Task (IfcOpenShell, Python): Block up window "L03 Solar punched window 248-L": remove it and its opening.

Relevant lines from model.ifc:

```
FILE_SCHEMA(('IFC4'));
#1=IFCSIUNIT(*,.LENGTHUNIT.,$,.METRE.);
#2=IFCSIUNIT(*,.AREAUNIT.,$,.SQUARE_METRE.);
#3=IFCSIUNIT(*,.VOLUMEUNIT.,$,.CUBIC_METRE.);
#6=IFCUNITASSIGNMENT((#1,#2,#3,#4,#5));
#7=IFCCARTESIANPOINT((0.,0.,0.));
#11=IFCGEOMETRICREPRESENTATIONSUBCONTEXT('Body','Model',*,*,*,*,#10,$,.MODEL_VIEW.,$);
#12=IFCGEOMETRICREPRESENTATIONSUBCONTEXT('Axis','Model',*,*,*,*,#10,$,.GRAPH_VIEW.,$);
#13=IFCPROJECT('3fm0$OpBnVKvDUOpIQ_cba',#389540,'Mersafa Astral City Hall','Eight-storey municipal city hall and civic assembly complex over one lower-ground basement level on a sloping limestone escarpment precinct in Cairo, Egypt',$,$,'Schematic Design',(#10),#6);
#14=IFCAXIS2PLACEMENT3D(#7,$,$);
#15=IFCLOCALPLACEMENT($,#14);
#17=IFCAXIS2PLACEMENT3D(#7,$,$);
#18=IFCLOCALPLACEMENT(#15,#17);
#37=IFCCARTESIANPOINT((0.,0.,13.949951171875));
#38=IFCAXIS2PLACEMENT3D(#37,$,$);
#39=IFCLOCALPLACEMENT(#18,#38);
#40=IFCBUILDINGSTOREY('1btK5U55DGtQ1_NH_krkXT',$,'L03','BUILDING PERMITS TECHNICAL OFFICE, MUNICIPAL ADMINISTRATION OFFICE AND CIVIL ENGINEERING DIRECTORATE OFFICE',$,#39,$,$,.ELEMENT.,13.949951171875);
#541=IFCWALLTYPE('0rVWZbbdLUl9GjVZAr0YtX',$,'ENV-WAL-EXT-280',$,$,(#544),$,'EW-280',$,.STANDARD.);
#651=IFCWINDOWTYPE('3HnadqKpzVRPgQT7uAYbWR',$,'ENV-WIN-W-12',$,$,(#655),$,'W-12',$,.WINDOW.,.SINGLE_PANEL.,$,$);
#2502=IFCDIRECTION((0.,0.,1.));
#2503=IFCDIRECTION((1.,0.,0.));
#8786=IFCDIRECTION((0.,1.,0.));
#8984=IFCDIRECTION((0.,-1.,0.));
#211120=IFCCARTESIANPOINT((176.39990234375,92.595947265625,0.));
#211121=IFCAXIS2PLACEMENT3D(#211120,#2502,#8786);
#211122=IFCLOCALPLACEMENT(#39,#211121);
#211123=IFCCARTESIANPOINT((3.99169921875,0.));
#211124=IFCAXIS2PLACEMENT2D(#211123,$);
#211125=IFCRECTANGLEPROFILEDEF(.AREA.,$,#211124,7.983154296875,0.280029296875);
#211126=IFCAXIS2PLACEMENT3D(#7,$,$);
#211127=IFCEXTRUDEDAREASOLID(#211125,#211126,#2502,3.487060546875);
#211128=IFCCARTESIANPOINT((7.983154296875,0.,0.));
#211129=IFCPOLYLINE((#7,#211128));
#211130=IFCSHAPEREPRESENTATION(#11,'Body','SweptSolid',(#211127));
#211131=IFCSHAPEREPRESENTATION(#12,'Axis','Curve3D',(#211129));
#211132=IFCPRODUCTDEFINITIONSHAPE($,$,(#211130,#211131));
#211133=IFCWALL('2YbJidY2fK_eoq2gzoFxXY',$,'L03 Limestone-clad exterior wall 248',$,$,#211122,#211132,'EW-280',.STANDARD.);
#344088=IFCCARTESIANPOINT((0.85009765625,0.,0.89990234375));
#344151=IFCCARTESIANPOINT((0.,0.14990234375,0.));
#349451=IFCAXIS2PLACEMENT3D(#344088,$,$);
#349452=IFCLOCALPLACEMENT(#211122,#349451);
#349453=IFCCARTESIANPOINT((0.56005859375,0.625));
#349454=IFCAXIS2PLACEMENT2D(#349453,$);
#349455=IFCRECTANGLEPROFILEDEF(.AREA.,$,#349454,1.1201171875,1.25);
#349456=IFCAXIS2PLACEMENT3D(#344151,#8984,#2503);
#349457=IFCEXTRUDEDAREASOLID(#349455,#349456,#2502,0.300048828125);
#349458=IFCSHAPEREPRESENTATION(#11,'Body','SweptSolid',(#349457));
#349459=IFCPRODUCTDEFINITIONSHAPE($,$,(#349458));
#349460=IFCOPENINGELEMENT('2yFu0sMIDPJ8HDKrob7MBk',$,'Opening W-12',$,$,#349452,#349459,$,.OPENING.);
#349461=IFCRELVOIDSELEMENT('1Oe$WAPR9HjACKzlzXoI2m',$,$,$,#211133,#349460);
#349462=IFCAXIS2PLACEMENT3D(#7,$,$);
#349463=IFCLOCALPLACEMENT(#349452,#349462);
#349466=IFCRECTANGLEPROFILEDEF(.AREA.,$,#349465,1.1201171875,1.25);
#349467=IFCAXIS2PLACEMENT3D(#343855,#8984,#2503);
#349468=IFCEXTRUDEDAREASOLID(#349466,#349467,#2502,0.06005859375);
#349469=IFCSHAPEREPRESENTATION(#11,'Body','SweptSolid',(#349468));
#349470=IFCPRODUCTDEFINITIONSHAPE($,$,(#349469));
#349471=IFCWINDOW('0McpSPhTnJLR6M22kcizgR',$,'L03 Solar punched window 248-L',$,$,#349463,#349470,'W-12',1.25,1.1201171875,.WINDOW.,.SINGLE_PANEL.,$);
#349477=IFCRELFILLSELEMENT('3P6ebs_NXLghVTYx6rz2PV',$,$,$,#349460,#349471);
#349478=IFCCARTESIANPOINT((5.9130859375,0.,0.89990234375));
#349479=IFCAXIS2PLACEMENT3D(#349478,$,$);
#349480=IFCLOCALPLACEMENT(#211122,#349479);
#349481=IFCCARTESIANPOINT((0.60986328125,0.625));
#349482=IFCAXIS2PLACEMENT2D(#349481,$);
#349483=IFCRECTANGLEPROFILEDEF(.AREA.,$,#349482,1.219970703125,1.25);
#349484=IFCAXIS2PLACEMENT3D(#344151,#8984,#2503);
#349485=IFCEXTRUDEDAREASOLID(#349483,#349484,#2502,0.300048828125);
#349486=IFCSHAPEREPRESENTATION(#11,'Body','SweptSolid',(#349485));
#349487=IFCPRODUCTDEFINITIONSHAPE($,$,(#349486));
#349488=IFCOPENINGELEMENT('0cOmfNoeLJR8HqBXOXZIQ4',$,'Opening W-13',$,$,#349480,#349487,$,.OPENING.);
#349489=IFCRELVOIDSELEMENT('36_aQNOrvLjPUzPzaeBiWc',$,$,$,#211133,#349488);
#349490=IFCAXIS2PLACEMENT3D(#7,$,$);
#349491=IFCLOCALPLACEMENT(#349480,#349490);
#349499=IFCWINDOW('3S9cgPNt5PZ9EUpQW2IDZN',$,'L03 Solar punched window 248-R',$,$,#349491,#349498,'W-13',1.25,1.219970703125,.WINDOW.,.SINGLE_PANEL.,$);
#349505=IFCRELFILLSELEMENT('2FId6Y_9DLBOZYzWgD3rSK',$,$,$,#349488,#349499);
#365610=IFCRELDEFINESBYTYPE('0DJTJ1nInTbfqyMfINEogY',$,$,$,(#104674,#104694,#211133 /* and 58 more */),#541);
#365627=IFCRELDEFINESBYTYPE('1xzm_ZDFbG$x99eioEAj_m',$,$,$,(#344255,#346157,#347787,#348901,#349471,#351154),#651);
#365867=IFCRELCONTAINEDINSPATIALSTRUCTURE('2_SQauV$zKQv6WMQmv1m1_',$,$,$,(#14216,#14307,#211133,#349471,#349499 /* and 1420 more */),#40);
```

```python
import ifcopenshell
import ifcopenshell.api.feature
import ifcopenshell.api.root
import ifcopenshell.geom
import ifcopenshell.util.shape

model = ifcopenshell.open("model.ifc")
settings = ifcopenshell.geom.settings()


def volume(element):
    """Net volume in cubic metres, openings subtracted."""
    shape = ifcopenshell.geom.create_shape(settings, element)
    return ifcopenshell.util.shape.get_volume(shape.geometry)


window = model.by_guid("0McpSPhTnJLR6M22kcizgR")
opening = window.FillsVoids[0].RelatingOpeningElement
wall = opening.VoidsElements[0].RelatingBuildingElement
before = volume(wall)

ifcopenshell.api.root.remove_product(model, product=window)
ifcopenshell.api.feature.remove_feature(model, feature=opening)

after = volume(wall)

print(f"wall volume {before:.3f} -> {after:.3f} m3")

model.write("model_v2.ifc")
```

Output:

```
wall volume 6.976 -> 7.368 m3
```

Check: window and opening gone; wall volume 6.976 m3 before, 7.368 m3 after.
